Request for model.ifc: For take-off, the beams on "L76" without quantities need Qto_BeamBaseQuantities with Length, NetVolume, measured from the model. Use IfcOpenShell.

First a look at what the model holds.

```python
import ifcopenshell
import ifcopenshell.util.element
import ifcopenshell.util.unit

model = ifcopenshell.open("model.ifc")
print(model.schema)
for unit_type in ("LENGTHUNIT", "AREAUNIT", "VOLUMEUNIT"):
    print(unit_type, ifcopenshell.util.unit.calculate_unit_scale(model, unit_type))
storey = next(s for s in model.by_type("IfcBuildingStorey") if s.Name == "L76")
beams = [e for e in ifcopenshell.util.element.get_decomposition(storey) if e.is_a("IfcBeam")]
for e in sorted(beams, key=lambda e: e.id()):
    print(e.id(), e.is_a(), e.Name, list(ifcopenshell.util.element.get_psets(e, qtos_only=True)), sep=" | ")
```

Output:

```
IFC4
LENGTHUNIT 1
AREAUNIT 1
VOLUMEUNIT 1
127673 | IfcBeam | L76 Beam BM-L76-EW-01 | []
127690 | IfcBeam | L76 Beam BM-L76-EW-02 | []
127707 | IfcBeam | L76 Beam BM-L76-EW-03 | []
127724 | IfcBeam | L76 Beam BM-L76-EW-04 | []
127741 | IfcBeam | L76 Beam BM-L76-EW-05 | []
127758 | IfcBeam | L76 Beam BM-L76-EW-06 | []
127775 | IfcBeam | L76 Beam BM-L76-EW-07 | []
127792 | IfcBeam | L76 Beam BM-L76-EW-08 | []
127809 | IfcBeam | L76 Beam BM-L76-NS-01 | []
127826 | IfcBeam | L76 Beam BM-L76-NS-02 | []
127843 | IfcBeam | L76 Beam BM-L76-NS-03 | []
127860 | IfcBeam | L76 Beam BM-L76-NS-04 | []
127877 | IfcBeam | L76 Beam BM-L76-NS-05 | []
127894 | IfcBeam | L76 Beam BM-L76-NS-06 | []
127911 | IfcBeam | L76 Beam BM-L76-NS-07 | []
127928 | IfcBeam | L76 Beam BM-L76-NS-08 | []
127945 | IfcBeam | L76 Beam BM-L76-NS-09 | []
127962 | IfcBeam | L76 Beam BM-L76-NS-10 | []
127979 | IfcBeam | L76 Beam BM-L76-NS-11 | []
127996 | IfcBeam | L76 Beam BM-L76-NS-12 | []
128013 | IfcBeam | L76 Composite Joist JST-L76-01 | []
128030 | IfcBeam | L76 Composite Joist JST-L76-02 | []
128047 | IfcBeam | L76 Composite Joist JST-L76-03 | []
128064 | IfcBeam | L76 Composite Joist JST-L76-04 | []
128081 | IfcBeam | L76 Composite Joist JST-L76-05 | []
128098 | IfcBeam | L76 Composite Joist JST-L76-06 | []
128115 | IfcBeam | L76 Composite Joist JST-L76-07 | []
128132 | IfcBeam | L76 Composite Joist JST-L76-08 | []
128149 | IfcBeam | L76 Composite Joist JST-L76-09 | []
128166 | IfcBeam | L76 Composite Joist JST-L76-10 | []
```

```python
import ifcopenshell
import ifcopenshell.api.pset
import ifcopenshell.geom
import ifcopenshell.util.element
import ifcopenshell.util.shape
import ifcopenshell.util.unit

model = ifcopenshell.open("model.ifc")
unit_scale = ifcopenshell.util.unit.calculate_unit_scale(model)
volume_scale = ifcopenshell.util.unit.calculate_unit_scale(model, "VOLUMEUNIT")
settings = ifcopenshell.geom.settings()

storey = next(s for s in model.by_type("IfcBuildingStorey") if s.Name == "L76")
beams = [e for e in ifcopenshell.util.element.get_decomposition(storey) if e.is_a("IfcBeam")]

for e in sorted(beams, key=lambda e: e.id()):
    if ifcopenshell.util.element.get_psets(e, qtos_only=True, should_inherit=False):
        continue
    # Geometry comes back in metres, in the element's own axes.
    shape = ifcopenshell.geom.create_shape(settings, e)
    values = {
        "Length": ifcopenshell.util.shape.get_max_xyz(shape.geometry) / unit_scale,
        "NetVolume": ifcopenshell.util.shape.get_volume(shape.geometry) / volume_scale,
    }
    qto = ifcopenshell.api.pset.add_qto(model, product=e, name="Qto_BeamBaseQuantities")
    ifcopenshell.api.pset.edit_qto(model, qto=qto, properties=values)
    print(e.id(), {k: round(v, 3) for k, v in values.items()})

model.write("model_edited.ifc")
```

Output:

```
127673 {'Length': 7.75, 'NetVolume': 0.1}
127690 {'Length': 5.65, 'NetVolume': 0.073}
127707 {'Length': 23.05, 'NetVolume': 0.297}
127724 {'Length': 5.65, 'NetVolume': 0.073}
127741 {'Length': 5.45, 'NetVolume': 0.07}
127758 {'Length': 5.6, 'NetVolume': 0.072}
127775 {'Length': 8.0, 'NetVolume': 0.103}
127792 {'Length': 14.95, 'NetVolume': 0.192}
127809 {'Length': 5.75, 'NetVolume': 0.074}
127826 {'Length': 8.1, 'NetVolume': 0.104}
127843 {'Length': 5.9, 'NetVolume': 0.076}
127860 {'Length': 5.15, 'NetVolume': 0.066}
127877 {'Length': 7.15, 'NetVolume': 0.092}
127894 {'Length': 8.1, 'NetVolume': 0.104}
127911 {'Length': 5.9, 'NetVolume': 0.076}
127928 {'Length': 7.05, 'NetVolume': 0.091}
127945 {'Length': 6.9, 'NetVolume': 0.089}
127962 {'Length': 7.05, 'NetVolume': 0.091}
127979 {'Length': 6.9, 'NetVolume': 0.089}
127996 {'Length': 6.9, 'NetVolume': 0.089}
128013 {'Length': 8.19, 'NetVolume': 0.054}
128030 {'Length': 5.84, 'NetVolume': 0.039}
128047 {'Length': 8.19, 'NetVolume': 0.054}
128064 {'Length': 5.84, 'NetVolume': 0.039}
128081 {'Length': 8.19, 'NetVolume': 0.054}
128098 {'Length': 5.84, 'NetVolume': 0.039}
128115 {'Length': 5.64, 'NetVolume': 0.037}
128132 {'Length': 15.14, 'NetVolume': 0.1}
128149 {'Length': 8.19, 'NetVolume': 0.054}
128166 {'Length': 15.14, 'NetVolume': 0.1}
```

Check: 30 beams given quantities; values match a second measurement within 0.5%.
